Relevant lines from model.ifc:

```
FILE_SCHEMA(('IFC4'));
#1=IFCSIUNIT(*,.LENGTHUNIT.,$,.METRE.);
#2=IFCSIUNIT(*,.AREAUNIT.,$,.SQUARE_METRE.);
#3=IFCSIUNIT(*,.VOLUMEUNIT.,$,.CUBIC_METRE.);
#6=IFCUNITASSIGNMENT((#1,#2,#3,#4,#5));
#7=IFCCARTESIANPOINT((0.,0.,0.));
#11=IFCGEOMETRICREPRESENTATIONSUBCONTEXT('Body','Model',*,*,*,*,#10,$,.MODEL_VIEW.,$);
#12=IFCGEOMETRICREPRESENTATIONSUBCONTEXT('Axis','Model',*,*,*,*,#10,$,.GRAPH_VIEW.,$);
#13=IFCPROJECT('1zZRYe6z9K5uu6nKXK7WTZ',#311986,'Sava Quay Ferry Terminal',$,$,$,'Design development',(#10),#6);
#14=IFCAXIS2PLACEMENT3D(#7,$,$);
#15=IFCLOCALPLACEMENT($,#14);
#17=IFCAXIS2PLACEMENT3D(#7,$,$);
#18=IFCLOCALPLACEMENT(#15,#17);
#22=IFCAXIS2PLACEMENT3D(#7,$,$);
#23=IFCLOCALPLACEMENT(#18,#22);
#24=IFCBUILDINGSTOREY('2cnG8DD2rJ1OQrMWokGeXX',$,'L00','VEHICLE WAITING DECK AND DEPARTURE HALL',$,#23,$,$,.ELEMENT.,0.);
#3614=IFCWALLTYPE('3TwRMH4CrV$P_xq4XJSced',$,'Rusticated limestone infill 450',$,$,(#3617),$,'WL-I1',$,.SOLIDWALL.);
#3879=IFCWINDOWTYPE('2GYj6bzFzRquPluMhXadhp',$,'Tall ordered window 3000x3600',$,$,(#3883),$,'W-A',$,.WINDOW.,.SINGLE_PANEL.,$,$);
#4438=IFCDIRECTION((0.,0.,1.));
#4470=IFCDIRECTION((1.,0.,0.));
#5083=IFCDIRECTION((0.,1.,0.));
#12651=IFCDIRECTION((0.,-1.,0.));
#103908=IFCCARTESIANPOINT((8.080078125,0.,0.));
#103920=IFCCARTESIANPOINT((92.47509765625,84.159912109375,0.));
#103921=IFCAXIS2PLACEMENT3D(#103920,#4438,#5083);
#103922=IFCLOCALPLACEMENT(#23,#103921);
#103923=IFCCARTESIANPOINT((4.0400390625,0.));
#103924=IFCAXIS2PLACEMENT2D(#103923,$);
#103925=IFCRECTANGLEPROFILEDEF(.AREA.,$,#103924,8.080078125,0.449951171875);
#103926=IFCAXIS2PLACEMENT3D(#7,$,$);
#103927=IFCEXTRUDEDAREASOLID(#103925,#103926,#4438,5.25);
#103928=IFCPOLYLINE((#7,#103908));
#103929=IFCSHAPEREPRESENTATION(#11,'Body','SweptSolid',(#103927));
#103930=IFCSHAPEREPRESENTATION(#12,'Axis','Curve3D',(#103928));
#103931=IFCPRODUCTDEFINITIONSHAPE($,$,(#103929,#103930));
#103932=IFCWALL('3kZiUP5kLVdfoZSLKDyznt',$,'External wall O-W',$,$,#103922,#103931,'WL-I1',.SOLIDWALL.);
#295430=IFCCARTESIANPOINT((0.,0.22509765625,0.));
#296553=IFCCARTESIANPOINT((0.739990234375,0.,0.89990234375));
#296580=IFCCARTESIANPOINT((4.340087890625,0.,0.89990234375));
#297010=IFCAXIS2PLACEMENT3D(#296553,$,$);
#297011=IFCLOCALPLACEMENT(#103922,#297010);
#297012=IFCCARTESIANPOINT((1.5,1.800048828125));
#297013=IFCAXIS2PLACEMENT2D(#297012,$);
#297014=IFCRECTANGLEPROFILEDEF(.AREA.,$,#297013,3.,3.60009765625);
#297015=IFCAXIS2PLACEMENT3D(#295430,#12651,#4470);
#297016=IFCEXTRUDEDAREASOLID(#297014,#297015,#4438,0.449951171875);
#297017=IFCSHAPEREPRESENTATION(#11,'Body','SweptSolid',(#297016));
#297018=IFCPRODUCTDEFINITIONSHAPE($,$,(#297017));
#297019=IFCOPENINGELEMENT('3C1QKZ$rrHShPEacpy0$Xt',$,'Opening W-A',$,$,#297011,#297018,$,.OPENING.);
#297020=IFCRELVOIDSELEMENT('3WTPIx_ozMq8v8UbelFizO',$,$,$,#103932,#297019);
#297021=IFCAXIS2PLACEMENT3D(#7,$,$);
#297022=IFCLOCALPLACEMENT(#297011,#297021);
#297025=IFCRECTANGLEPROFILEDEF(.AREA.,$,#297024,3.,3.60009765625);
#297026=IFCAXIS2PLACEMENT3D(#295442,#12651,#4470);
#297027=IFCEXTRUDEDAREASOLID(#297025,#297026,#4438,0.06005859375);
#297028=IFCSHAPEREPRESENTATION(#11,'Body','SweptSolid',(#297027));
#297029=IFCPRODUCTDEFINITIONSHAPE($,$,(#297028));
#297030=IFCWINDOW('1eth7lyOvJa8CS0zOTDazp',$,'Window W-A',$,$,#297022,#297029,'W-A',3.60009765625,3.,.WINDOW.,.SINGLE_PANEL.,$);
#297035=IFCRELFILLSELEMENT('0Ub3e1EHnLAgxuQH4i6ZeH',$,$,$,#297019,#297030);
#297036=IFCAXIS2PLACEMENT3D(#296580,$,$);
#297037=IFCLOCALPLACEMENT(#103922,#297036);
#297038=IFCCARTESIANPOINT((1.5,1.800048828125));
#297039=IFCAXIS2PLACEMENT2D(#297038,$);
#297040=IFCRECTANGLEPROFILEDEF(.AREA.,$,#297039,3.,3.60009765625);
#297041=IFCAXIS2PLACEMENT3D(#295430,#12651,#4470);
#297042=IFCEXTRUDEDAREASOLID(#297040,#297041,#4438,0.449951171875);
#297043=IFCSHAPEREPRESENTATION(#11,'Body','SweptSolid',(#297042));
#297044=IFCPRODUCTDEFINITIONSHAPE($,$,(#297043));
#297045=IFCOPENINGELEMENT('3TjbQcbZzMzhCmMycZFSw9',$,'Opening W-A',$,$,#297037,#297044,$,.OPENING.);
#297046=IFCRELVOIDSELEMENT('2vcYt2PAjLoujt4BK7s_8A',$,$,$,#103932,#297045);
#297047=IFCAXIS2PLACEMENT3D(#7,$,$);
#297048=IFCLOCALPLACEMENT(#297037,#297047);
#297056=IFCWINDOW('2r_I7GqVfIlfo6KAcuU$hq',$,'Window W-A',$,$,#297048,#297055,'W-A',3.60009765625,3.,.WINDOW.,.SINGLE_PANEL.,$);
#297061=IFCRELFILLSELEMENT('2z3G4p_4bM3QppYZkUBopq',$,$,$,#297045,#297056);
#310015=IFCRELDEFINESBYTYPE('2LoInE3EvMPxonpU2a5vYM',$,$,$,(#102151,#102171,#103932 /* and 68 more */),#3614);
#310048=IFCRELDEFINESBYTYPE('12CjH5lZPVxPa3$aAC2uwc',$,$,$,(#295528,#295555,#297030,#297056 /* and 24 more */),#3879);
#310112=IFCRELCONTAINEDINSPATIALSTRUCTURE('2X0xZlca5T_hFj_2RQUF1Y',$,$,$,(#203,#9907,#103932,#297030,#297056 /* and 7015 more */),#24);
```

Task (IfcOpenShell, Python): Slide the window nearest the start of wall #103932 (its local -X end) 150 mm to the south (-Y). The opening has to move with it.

```python
import ifcopenshell
import ifcopenshell.api.geometry
import ifcopenshell.util.placement

model = ifcopenshell.open("model.ifc")

window = model.by_guid("1eth7lyOvJa8CS0zOTDazp")
opening = window.FillsVoids[0].RelatingOpeningElement
wall = opening.VoidsElements[0].RelatingBuildingElement

wall_matrix = ifcopenshell.util.placement.get_local_placement(wall.ObjectPlacement)
shift = wall_matrix[:3, 0] * -0.15
before = ifcopenshell.util.placement.get_local_placement(window.ObjectPlacement)[:3, 3].copy()

# The window is placed relative to its opening, so it follows when the opening moves.
matrix = ifcopenshell.util.placement.get_local_placement(opening.ObjectPlacement)
matrix[:3, 3] += shift
ifcopenshell.api.geometry.edit_object_placement(
    model, product=opening, matrix=matrix, is_si=False, should_transform_children=True
)

after = ifcopenshell.util.placement.get_local_placement(window.ObjectPlacement)[:3, 3]
print("window moved by", (after - before).round(3) + 0.0)

model.write("model_v2.ifc")
```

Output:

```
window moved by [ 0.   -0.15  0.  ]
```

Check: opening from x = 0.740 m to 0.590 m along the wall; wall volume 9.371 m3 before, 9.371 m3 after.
